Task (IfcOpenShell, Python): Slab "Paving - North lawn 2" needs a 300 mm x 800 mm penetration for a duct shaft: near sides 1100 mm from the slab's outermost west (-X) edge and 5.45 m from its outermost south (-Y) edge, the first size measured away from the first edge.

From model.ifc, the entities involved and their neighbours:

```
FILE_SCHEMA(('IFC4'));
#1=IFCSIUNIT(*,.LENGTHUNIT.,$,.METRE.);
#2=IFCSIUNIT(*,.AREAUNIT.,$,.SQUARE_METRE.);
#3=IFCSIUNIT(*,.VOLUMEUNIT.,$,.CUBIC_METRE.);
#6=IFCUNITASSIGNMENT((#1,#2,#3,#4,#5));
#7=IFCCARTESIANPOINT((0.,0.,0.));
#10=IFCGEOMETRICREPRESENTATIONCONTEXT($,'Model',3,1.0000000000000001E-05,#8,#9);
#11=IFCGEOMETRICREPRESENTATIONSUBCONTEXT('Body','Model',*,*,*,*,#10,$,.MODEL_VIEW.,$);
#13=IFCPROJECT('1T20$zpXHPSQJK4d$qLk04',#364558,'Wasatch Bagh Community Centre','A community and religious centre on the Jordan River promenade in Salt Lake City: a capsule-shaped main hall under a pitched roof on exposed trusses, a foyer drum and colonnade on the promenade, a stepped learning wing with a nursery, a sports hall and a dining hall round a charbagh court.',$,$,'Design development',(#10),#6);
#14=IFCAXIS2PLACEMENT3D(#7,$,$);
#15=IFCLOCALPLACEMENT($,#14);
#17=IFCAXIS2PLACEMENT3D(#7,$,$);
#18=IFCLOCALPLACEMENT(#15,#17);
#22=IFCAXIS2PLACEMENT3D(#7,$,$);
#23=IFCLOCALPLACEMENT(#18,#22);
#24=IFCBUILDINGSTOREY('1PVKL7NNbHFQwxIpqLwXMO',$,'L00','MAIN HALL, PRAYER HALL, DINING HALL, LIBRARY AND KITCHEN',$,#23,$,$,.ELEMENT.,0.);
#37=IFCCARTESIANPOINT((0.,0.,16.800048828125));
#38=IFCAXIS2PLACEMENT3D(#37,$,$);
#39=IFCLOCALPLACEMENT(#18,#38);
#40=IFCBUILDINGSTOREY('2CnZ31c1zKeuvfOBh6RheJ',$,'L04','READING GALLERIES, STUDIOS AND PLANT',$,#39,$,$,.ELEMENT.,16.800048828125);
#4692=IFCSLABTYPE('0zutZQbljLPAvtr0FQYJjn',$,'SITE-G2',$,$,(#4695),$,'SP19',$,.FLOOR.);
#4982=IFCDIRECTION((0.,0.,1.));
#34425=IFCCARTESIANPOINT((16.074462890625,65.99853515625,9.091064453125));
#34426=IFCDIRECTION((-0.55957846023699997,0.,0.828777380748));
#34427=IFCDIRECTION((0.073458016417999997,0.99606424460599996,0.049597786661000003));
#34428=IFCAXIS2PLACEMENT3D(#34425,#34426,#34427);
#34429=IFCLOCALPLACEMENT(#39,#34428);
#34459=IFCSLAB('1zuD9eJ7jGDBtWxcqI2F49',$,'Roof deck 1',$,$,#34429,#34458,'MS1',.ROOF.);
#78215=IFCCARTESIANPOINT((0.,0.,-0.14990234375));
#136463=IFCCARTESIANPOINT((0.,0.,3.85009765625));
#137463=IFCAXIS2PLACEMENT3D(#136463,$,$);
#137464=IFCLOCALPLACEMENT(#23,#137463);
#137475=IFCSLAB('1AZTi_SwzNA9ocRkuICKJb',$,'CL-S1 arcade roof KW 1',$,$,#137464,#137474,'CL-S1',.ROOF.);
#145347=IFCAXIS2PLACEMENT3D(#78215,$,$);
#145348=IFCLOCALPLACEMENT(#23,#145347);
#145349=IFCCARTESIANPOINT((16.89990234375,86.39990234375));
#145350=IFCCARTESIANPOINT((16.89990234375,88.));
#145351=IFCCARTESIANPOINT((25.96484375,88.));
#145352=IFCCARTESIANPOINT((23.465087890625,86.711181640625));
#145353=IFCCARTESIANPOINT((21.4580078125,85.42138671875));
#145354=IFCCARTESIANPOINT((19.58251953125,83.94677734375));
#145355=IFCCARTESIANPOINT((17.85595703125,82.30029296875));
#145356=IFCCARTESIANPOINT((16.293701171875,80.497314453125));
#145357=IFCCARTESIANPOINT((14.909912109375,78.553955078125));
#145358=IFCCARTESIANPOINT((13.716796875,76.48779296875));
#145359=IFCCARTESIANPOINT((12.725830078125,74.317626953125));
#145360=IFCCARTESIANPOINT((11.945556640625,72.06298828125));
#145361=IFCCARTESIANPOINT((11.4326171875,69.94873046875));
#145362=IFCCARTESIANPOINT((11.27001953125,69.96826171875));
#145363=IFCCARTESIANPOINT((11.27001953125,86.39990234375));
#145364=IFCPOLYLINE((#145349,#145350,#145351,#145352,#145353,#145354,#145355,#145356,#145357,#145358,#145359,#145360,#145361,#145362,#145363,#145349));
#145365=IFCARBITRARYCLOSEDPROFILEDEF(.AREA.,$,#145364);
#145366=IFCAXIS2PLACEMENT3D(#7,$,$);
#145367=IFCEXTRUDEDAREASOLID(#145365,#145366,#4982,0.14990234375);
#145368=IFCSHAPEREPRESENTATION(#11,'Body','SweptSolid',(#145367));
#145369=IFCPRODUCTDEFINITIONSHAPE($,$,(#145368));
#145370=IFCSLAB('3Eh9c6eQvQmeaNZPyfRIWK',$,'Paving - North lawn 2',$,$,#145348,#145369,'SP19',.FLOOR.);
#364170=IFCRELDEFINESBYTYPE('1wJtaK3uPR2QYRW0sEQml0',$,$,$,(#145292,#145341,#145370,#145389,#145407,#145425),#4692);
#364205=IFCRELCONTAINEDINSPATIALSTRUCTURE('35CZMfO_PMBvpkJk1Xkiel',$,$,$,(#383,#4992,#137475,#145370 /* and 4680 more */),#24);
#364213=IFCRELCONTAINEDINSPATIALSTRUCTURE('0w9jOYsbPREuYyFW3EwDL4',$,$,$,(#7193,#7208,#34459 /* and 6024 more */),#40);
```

```python
import numpy as np
import ifcopenshell
import ifcopenshell.api.feature
import ifcopenshell.api.geometry
import ifcopenshell.api.root
import ifcopenshell.geom
import ifcopenshell.util.placement
import ifcopenshell.util.representation
import ifcopenshell.util.shape
import ifcopenshell.util.unit

model = ifcopenshell.open("model.ifc")
unit_scale = ifcopenshell.util.unit.calculate_unit_scale(model)
settings = ifcopenshell.geom.settings()


def volume(element):
    """Net volume in cubic metres, openings subtracted."""
    shape = ifcopenshell.geom.create_shape(settings, element)
    return ifcopenshell.util.shape.get_volume(shape.geometry)


slab = model.by_guid("3Eh9c6eQvQmeaNZPyfRIWK")
before = volume(slab)

# Extent in the slab's own axes, in metres. The edges named are its -X and -Y sides.
slab_shape = ifcopenshell.geom.create_shape(settings, slab)
vertices = ifcopenshell.util.shape.get_vertices(slab_shape.geometry)
x_min, y_min, bottom = vertices.min(axis=0)
top = vertices[:, 2].max()

opening = ifcopenshell.api.root.create_entity(model, ifc_class="IfcOpeningElement", name="Duct shaft opening", predefined_type="OPENING")
context = ifcopenshell.util.representation.get_context(model, "Model", "Body", "MODEL_VIEW")
width, depth = 0.3, 0.8
outline = [(0.0, 0.0), (width, 0.0), (width, depth), (0.0, depth), (0.0, 0.0)]
# Overshoot both faces by 50 mm so the cut is clean.
shape = ifcopenshell.api.geometry.add_slab_representation(
    model, context=context, depth=top - bottom + 0.1, polyline=outline
)
ifcopenshell.api.geometry.assign_representation(model, product=opening, representation=shape)

matrix = ifcopenshell.util.placement.get_local_placement(slab.ObjectPlacement)
matrix[:, 3] = matrix @ np.append(np.array([x_min + 1.1, y_min + 5.45, bottom - 0.05]) / unit_scale, 1.0)
ifcopenshell.api.geometry.edit_object_placement(model, product=opening, matrix=matrix, is_si=False)
ifcopenshell.api.feature.add_feature(model, feature=opening, element=slab)

after = volume(slab)

print(f"slab volume {before:.3f} -> {after:.3f} m3")

model.write("model-out.ifc")
```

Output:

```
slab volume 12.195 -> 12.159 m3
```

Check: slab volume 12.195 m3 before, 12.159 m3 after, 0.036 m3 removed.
